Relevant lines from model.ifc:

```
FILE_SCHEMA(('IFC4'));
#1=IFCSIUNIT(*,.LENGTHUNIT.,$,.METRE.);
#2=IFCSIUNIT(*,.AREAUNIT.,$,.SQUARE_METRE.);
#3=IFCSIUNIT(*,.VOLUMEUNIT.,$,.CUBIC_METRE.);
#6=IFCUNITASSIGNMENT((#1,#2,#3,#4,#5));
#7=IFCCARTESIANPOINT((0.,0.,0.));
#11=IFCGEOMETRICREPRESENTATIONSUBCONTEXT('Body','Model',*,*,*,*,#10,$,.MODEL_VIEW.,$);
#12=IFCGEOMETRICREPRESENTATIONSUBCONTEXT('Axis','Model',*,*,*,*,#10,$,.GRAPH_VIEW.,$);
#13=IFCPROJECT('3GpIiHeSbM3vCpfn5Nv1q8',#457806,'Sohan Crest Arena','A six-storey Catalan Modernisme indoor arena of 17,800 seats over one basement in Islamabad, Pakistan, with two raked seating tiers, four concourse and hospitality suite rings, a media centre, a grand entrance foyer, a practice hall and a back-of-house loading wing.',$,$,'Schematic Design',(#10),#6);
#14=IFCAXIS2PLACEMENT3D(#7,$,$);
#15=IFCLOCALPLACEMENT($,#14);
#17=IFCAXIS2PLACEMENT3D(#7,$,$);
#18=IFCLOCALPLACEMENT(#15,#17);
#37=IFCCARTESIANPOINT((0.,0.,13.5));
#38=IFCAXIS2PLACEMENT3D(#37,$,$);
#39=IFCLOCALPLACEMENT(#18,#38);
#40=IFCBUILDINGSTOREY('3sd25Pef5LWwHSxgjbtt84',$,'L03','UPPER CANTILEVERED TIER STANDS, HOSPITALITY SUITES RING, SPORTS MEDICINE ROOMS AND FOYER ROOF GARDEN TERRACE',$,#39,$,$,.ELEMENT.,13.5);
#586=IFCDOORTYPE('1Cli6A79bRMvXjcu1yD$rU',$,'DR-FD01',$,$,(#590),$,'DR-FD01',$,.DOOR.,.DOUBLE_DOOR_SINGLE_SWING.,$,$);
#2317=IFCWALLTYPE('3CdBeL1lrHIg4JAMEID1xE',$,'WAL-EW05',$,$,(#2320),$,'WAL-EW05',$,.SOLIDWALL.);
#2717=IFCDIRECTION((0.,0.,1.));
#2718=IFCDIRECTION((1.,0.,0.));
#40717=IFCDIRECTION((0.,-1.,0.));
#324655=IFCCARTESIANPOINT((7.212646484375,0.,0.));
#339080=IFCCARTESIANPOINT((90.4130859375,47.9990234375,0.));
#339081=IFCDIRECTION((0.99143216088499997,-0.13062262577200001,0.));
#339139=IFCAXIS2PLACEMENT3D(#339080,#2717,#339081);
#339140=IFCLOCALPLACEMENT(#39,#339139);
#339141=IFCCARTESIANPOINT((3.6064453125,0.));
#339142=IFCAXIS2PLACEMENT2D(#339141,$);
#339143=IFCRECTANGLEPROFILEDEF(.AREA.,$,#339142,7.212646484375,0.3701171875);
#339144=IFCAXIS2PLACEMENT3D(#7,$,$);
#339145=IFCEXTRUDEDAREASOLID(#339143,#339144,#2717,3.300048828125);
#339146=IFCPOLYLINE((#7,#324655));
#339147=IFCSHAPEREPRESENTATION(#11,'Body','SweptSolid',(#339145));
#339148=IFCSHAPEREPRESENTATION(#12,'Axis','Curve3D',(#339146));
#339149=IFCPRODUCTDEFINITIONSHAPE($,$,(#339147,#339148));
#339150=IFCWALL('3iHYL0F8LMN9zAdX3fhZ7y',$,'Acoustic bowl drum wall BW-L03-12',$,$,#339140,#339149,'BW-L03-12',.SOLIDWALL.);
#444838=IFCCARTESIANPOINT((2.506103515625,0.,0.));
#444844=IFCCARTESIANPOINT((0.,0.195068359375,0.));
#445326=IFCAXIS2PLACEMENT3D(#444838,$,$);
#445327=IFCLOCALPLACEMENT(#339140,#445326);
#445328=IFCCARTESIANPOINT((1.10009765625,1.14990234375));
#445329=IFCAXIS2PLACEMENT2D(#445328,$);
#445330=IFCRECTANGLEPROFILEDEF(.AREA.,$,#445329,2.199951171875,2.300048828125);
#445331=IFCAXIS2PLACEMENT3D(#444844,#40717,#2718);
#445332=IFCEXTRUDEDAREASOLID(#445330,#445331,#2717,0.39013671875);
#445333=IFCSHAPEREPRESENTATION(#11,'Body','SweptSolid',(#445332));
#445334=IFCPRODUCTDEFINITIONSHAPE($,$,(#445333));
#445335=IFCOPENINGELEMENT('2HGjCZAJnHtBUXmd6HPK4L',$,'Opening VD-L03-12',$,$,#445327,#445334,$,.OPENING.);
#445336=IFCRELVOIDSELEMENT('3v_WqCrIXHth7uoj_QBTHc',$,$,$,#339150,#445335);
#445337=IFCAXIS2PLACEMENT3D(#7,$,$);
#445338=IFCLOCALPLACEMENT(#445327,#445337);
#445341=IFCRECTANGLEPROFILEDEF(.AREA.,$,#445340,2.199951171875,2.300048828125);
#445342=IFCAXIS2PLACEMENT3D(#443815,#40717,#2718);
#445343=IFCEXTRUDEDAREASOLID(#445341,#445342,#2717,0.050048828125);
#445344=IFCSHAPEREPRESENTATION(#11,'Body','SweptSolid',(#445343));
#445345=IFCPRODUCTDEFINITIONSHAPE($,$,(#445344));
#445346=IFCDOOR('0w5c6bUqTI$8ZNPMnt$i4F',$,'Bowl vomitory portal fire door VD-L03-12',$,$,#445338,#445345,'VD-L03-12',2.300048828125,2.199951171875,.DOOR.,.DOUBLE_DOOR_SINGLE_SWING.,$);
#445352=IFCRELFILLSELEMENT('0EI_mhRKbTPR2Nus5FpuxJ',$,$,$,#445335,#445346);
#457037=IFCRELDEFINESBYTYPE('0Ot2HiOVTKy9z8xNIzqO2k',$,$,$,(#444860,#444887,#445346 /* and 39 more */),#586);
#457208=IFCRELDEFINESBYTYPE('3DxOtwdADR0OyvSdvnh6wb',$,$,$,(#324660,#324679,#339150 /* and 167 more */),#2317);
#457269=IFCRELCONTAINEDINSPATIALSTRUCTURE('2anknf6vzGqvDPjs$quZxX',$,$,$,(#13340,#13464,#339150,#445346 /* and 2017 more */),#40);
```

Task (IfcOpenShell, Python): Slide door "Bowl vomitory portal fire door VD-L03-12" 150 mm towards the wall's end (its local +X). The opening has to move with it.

```python
import ifcopenshell
import ifcopenshell.api.geometry
import ifcopenshell.util.placement
import ifcopenshell.util.unit

model = ifcopenshell.open("model.ifc")
unit_scale = ifcopenshell.util.unit.calculate_unit_scale(model)

door = model.by_guid("0w5c6bUqTI$8ZNPMnt$i4F")
opening = door.FillsVoids[0].RelatingOpeningElement
wall = opening.VoidsElements[0].RelatingBuildingElement

wall_matrix = ifcopenshell.util.placement.get_local_placement(wall.ObjectPlacement)
shift = wall_matrix[:3, 0] * 0.15 / unit_scale
before = ifcopenshell.util.placement.get_local_placement(door.ObjectPlacement)[:3, 3].copy()

# The door is placed relative to its opening, so it follows when the opening moves.
matrix = ifcopenshell.util.placement.get_local_placement(opening.ObjectPlacement)
matrix[:3, 3] += shift
ifcopenshell.api.geometry.edit_object_placement(
    model, product=opening, matrix=matrix, is_si=False, should_transform_children=True
)

after = ifcopenshell.util.placement.get_local_placement(door.ObjectPlacement)[:3, 3]
print("door moved by", (after - before).round(3) + 0.0)

model.write("model_edited.ifc")
```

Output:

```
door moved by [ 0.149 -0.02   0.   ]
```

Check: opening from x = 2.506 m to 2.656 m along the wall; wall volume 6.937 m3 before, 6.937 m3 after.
